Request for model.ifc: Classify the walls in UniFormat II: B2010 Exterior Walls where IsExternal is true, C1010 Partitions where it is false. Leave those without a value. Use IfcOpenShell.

First a look at what the model holds.

```python
import ifcopenshell
import ifcopenshell.util.element

model = ifcopenshell.open("model.ifc")
print(model.schema)
print("classifications:", [c.Name for c in model.by_type("IfcClassification")])
values = [ifcopenshell.util.element.get_pset(e, "Pset_WallCommon", "IsExternal") for e in model.by_type("IfcWall")]
for value in (True, False, None):
    print("IsExternal", value, values.count(value))
```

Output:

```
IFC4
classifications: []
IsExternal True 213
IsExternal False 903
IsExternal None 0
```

```python
import ifcopenshell
import ifcopenshell.api.classification
import ifcopenshell.util.element

model = ifcopenshell.open("model.ifc")

system = ifcopenshell.api.classification.add_classification(model, classification="UniFormat II")

walls = model.by_type("IfcWall")
external = {e: ifcopenshell.util.element.get_pset(e, "Pset_WallCommon", "IsExternal") for e in walls}
for flag, code, name in ((True, "B2010", "Exterior Walls"), (False, "C1010", "Partitions")):
    products = [e for e in walls if external[e] is flag]
    ifcopenshell.api.classification.add_reference(
        model, products=products, classification=system, identification=code, name=name
    )
    print(code, len(products))

model.write("model_edited.ifc")
```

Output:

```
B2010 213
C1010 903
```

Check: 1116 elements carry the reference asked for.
